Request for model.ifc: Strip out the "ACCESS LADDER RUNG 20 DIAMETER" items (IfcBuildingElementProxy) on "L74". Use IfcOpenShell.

First a look at what the model holds.

```python
import ifcopenshell
import ifcopenshell.util.element

model = ifcopenshell.open("model.ifc")
print(model.schema)
storey = next(s for s in model.by_type("IfcBuildingStorey") if s.Name == "L74")
proxies = [e for e in ifcopenshell.util.element.get_decomposition(storey) if e.is_a("IfcBuildingElementProxy")]
seen = {}
for e in proxies:
    element_type = ifcopenshell.util.element.get_type(e)
    name = element_type.Name if element_type not in (None, e) else None
    seen[name] = seen.get(name, 0) + 1
for name, count in sorted(seen.items(), key=str):
    print(count, "x", name)
```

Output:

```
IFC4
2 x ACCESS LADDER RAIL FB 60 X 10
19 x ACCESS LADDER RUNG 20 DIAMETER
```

```python
import ifcopenshell
import ifcopenshell.api.root
import ifcopenshell.util.element

model = ifcopenshell.open("model.ifc")

storey = next(s for s in model.by_type("IfcBuildingStorey") if s.Name == "L74")
proxies = [e for e in ifcopenshell.util.element.get_decomposition(storey) if e.is_a("IfcBuildingElementProxy")]
targets = [e for e in proxies if (t := ifcopenshell.util.element.get_type(e)) not in (None, e) and t.Name == "ACCESS LADDER RUNG 20 DIAMETER"]

for e in targets:
    ifcopenshell.api.root.remove_product(model, product=e)
print(len(targets), "removed")

model.write("model_v2.ifc")
```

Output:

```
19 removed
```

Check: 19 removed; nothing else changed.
